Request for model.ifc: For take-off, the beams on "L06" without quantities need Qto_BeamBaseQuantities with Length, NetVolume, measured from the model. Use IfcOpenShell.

First a look at what the model holds.

```python
import ifcopenshell
import ifcopenshell.util.element
import ifcopenshell.util.unit

model = ifcopenshell.open("model.ifc")
print(model.schema)
for unit_type in ("LENGTHUNIT", "AREAUNIT", "VOLUMEUNIT"):
    print(unit_type, ifcopenshell.util.unit.calculate_unit_scale(model, unit_type))
storey = next(s for s in model.by_type("IfcBuildingStorey") if s.Name == "L06")
beams = [e for e in ifcopenshell.util.element.get_decomposition(storey) if e.is_a("IfcBeam")]
for e in sorted(beams, key=lambda e: e.id()):
    print(e.id(), e.is_a(), e.Name, list(ifcopenshell.util.element.get_psets(e, qtos_only=True)), sep=" | ")
```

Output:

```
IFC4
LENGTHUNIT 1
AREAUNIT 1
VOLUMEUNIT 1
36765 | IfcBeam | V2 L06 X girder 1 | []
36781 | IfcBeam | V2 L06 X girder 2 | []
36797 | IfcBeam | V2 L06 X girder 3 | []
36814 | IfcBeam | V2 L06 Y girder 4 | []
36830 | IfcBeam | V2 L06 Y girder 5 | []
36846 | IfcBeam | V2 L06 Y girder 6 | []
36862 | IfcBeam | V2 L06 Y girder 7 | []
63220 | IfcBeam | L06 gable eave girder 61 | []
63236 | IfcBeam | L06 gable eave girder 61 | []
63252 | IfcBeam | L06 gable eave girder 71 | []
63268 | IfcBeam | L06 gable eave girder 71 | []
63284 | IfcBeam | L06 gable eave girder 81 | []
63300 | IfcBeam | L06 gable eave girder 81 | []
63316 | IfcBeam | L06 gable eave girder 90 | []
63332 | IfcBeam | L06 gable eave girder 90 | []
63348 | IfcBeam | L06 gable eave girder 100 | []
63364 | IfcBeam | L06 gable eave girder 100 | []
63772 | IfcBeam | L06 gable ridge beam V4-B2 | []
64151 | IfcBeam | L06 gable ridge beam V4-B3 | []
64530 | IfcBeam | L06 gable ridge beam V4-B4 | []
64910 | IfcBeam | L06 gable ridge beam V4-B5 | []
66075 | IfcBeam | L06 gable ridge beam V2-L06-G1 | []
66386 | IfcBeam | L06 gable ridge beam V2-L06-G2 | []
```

```python
import ifcopenshell
import ifcopenshell.api.pset
import ifcopenshell.geom
import ifcopenshell.util.element
import ifcopenshell.util.shape
import ifcopenshell.util.unit

model = ifcopenshell.open("model.ifc")
unit_scale = ifcopenshell.util.unit.calculate_unit_scale(model)
volume_scale = ifcopenshell.util.unit.calculate_unit_scale(model, "VOLUMEUNIT")
settings = ifcopenshell.geom.settings()

storey = next(s for s in model.by_type("IfcBuildingStorey") if s.Name == "L06")
beams = [e for e in ifcopenshell.util.element.get_decomposition(storey) if e.is_a("IfcBeam")]

for e in sorted(beams, key=lambda e: e.id()):
    if ifcopenshell.util.element.get_psets(e, qtos_only=True, should_inherit=False):
        continue
    # Geometry comes back in metres, in the element's own axes.
    shape = ifcopenshell.geom.create_shape(settings, e)
    values = {
        "Length": ifcopenshell.util.shape.get_max_xyz(shape.geometry) / unit_scale,
        "NetVolume": ifcopenshell.util.shape.get_volume(shape.geometry) / volume_scale,
    }
    qto = ifcopenshell.api.pset.add_qto(model, product=e, name="Qto_BeamBaseQuantities")
    ifcopenshell.api.pset.edit_qto(model, qto=qto, properties=values)
    print(e.id(), {k: round(v, 3) for k, v in values.items()})

model.write("model_v2.ifc")
```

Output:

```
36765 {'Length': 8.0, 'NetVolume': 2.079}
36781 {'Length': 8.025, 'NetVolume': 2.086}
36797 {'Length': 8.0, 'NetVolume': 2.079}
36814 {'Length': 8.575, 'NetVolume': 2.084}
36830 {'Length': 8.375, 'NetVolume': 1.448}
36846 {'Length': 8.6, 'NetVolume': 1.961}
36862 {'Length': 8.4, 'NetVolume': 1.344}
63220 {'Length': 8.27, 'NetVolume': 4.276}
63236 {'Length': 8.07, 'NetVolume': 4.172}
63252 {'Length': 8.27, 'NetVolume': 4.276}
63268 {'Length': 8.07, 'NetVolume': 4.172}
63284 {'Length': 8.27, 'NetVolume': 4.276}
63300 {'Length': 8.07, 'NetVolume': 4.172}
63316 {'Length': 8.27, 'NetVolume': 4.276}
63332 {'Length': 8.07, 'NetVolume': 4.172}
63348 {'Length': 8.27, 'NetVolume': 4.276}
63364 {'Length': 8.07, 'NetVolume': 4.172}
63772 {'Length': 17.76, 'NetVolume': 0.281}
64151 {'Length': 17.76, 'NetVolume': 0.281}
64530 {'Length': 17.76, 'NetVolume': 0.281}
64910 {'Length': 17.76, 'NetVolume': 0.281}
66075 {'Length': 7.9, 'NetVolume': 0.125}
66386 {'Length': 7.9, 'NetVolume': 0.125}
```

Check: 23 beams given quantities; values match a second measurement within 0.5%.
